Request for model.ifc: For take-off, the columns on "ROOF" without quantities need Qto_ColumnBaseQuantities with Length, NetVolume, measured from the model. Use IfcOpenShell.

First a look at what the model holds.

```python
import ifcopenshell
import ifcopenshell.util.element
import ifcopenshell.util.unit

model = ifcopenshell.open("model.ifc")
print(model.schema)
for unit_type in ("LENGTHUNIT", "AREAUNIT", "VOLUMEUNIT"):
    print(unit_type, ifcopenshell.util.unit.calculate_unit_scale(model, unit_type))
storey = next(s for s in model.by_type("IfcBuildingStorey") if s.Name == "ROOF")
columns = [e for e in ifcopenshell.util.element.get_decomposition(storey) if e.is_a("IfcColumn")]
for e in sorted(columns, key=lambda e: e.id()):
    print(e.id(), e.is_a(), e.Name, list(ifcopenshell.util.element.get_psets(e, qtos_only=True)), sep=" | ")
```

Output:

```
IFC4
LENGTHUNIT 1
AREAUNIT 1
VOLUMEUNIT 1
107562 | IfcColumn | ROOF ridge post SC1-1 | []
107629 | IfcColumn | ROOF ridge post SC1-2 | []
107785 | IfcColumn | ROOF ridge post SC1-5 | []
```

```python
import ifcopenshell
import ifcopenshell.api.pset
import ifcopenshell.geom
import ifcopenshell.util.element
import ifcopenshell.util.shape
import ifcopenshell.util.unit

model = ifcopenshell.open("model.ifc")
unit_scale = ifcopenshell.util.unit.calculate_unit_scale(model)
volume_scale = ifcopenshell.util.unit.calculate_unit_scale(model, "VOLUMEUNIT")
settings = ifcopenshell.geom.settings()

storey = next(s for s in model.by_type("IfcBuildingStorey") if s.Name == "ROOF")
columns = [e for e in ifcopenshell.util.element.get_decomposition(storey) if e.is_a("IfcColumn")]

for e in sorted(columns, key=lambda e: e.id()):
    if ifcopenshell.util.element.get_psets(e, qtos_only=True, should_inherit=False):
        continue
    # Geometry comes back in metres, in the element's own axes.
    shape = ifcopenshell.geom.create_shape(settings, e)
    values = {
        "Length": ifcopenshell.util.shape.get_z(shape.geometry) / unit_scale,
        "NetVolume": ifcopenshell.util.shape.get_volume(shape.geometry) / volume_scale,
    }
    qto = ifcopenshell.api.pset.add_qto(model, product=e, name="Qto_ColumnBaseQuantities")
    ifcopenshell.api.pset.edit_qto(model, qto=qto, properties=values)
    print(e.id(), {k: round(v, 3) for k, v in values.items()})

model.write("model_edited.ifc")
```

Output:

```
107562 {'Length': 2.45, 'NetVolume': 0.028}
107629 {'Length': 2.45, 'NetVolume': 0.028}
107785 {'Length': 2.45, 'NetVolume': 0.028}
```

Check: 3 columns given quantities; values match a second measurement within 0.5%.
